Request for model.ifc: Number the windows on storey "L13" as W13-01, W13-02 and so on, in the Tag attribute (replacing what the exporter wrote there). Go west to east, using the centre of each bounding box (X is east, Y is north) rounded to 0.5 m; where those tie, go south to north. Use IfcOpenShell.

First a look at what the model holds.

```python
import ifcopenshell
import ifcopenshell.util.element
import ifcopenshell.util.placement

model = ifcopenshell.open("model.ifc")
print(model.schema)
storey = next(s for s in model.by_type("IfcBuildingStorey") if s.Name == "L13")
windows = [e for e in ifcopenshell.util.element.get_decomposition(storey) if e.is_a("IfcWindow")]
for e in sorted(windows, key=lambda e: e.id()):
    origin = ifcopenshell.util.placement.get_local_placement(e.ObjectPlacement)[:3, 3]
    print(e.id(), e.Tag, e.Name, origin.round(2) + 0.0, sep=" | ")
```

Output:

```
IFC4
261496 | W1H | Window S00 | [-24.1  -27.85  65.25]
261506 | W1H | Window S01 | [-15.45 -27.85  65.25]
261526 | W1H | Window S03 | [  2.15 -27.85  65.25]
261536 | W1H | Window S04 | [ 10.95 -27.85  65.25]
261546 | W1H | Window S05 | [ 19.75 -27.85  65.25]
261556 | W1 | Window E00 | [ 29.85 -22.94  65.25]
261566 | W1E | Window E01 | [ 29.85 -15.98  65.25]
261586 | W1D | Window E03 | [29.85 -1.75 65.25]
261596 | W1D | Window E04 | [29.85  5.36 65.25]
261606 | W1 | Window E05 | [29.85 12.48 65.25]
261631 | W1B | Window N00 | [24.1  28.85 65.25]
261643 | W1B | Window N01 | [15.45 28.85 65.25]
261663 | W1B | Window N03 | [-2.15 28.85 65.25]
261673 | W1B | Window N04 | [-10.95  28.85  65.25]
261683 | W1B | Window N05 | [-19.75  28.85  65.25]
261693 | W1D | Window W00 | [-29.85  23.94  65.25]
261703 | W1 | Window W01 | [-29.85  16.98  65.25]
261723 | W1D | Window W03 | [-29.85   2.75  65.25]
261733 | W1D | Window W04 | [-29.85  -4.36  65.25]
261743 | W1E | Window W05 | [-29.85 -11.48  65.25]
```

```python
import ifcopenshell
import ifcopenshell.geom
import ifcopenshell.util.element
import ifcopenshell.util.shape

model = ifcopenshell.open("model.ifc")
settings = ifcopenshell.geom.settings()
settings.set("use-world-coords", True)


def centre(element):
    shape = ifcopenshell.geom.create_shape(settings, element)
    return ifcopenshell.util.shape.get_bbox_centroid(shape.geometry)


storey = next(s for s in model.by_type("IfcBuildingStorey") if s.Name == "L13")
windows = [e for e in ifcopenshell.util.element.get_decomposition(storey) if e.is_a("IfcWindow")]

# Insertion points can sit at a corner or the storey origin, so sort by the geometry (in metres).
centres = {e: centre(e) for e in windows}
windows.sort(key=lambda e: (round(centres[e][0] / 0.5), centres[e][1]))

for i, e in enumerate(windows, start=1):
    number = f"W13-{i:02d}"
    e.Tag = number
    print(e.id(), number)

model.write("model_updated.ifc")
```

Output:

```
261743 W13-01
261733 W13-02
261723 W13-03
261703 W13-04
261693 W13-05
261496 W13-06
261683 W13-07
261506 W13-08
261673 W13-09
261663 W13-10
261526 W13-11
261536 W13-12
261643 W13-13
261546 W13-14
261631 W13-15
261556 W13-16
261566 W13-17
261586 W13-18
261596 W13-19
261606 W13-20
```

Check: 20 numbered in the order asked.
